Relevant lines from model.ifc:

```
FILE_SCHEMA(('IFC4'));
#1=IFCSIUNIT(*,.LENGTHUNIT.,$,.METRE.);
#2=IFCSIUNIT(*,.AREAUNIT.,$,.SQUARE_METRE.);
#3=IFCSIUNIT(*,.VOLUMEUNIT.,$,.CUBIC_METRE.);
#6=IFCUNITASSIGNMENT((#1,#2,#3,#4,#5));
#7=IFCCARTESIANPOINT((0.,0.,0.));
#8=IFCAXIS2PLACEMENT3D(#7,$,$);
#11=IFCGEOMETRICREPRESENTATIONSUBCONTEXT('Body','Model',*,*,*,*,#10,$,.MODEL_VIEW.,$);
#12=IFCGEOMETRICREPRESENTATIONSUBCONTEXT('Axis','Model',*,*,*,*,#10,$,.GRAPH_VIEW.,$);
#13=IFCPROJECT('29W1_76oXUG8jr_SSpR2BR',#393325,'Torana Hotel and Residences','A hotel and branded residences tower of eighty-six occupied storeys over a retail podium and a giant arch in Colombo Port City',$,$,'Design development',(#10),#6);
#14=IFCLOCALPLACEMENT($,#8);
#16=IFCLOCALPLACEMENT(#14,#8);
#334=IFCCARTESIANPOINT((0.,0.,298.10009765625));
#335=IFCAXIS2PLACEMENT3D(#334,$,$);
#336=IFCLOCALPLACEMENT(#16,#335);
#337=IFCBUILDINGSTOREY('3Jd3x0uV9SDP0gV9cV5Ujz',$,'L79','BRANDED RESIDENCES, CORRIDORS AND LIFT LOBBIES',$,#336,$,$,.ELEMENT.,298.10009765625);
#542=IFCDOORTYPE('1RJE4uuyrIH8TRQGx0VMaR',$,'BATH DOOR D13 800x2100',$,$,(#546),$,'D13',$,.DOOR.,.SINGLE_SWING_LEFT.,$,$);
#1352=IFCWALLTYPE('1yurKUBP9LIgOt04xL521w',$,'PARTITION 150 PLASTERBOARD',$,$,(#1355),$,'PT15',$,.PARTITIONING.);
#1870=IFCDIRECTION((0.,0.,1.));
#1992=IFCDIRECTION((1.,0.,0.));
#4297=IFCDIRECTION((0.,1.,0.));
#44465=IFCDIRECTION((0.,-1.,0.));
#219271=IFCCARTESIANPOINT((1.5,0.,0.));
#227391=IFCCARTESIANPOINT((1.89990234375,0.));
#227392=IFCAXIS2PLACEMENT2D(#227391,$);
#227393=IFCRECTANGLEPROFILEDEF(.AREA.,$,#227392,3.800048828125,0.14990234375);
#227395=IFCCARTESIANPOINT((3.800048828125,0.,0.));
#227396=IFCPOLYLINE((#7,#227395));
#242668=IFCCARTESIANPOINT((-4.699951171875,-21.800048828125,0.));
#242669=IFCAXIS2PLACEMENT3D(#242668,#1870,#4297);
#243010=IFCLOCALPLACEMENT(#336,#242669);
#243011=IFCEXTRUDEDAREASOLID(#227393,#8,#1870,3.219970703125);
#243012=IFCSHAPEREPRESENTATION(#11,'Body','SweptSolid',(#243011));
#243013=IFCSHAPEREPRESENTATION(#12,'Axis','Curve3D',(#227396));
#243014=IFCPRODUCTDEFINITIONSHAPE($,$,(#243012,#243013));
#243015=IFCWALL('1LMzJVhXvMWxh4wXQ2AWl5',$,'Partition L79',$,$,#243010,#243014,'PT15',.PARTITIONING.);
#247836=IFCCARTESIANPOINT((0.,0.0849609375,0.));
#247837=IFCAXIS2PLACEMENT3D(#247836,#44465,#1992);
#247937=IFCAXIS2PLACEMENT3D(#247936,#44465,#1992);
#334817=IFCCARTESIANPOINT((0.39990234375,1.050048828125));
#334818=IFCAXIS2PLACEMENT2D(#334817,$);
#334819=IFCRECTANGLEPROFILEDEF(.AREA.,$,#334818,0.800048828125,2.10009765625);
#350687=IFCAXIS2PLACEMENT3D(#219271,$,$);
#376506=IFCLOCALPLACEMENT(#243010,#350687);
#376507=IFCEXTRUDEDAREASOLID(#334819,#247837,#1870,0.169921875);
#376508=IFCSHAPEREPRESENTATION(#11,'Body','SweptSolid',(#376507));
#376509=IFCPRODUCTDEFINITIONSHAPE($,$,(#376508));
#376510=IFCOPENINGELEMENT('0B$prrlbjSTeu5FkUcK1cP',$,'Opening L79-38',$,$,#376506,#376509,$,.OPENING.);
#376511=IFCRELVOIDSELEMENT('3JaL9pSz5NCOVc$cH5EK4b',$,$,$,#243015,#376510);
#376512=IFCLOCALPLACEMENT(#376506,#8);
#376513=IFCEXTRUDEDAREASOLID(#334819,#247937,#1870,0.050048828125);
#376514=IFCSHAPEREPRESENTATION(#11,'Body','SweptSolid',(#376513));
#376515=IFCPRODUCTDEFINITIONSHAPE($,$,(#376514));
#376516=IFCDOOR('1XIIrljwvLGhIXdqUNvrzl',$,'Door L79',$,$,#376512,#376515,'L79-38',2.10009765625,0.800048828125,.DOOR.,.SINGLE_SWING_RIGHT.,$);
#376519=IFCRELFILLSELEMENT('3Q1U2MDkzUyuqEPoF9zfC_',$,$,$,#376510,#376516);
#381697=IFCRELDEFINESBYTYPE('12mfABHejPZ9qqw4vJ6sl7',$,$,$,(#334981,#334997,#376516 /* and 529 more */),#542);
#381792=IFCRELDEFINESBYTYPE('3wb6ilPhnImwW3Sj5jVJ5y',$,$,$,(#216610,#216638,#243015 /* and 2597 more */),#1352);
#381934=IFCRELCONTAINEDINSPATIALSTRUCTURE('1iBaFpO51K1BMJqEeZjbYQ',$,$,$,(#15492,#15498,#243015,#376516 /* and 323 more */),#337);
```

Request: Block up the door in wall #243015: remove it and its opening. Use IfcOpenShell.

```python
import ifcopenshell
import ifcopenshell.api.feature
import ifcopenshell.api.root
import ifcopenshell.geom
import ifcopenshell.util.shape

model = ifcopenshell.open("model.ifc")
settings = ifcopenshell.geom.settings()


def volume(element):
    """Net volume in cubic metres, openings subtracted."""
    shape = ifcopenshell.geom.create_shape(settings, element)
    return ifcopenshell.util.shape.get_volume(shape.geometry)


door = model.by_id(376516)
opening = door.FillsVoids[0].RelatingOpeningElement
wall = opening.VoidsElements[0].RelatingBuildingElement
before = volume(wall)

ifcopenshell.api.root.remove_product(model, product=door)
ifcopenshell.api.feature.remove_feature(model, feature=opening)

after = volume(wall)

print(f"wall volume {before:.3f} -> {after:.3f} m3")

model.write("model_rev.ifc")
```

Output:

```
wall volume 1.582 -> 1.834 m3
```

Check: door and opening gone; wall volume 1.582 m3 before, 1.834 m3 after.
